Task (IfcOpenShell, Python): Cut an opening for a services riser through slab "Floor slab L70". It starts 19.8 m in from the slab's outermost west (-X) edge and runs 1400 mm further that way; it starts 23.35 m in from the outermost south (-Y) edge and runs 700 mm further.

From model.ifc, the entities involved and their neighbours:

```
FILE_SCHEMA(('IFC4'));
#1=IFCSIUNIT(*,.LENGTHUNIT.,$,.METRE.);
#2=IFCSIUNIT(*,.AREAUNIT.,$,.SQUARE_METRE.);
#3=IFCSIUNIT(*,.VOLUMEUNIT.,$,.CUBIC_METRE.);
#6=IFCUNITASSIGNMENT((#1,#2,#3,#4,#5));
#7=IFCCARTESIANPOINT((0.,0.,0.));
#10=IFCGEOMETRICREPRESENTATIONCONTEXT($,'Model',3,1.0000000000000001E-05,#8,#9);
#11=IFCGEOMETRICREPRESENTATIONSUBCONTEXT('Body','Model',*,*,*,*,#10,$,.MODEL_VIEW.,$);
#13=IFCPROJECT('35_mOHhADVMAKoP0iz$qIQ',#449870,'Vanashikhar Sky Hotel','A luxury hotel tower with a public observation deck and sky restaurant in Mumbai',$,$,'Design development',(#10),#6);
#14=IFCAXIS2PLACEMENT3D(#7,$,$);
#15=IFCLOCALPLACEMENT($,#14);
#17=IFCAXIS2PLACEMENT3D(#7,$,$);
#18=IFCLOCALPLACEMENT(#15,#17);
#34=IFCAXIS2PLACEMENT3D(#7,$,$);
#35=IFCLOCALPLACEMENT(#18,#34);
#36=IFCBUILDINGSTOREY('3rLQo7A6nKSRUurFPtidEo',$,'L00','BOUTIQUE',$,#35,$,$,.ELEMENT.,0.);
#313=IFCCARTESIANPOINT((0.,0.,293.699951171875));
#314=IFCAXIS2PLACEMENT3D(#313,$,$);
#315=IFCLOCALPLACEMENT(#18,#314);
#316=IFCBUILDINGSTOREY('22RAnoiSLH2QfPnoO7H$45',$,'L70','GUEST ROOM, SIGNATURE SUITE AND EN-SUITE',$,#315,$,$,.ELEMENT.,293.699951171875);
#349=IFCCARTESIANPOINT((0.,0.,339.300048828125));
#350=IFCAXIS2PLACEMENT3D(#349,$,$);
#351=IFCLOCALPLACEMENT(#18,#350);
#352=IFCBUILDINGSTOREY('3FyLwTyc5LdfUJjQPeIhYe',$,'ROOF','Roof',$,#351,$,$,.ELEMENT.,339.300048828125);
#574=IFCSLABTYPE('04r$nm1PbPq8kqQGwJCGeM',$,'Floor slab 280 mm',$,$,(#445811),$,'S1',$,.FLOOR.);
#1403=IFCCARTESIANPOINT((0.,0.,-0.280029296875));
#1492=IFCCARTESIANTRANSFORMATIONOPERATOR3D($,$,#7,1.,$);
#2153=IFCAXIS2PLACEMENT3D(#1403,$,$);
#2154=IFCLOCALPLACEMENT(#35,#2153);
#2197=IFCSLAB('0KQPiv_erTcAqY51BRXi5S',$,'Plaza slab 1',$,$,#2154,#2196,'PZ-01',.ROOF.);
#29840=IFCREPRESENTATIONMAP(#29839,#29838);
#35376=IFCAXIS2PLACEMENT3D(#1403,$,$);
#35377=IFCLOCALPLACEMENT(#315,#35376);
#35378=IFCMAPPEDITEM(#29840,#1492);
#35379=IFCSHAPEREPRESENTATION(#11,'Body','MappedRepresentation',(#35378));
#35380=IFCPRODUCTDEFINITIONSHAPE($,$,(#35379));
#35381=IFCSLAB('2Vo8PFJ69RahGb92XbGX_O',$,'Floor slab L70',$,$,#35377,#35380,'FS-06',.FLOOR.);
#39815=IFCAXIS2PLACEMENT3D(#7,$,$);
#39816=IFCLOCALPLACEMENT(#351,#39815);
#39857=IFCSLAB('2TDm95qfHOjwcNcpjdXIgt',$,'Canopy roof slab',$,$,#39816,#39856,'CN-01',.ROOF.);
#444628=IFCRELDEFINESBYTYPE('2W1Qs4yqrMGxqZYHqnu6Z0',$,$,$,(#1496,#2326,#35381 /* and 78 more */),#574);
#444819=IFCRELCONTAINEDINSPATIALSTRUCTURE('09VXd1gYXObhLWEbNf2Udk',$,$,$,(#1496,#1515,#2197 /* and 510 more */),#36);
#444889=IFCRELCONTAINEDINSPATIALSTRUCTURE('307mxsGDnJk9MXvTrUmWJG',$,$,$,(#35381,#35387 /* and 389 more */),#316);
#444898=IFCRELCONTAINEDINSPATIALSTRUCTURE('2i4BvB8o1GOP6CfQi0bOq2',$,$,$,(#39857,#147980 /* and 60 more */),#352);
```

```python
import numpy as np
import ifcopenshell
import ifcopenshell.api.feature
import ifcopenshell.api.geometry
import ifcopenshell.api.root
import ifcopenshell.geom
import ifcopenshell.util.placement
import ifcopenshell.util.representation
import ifcopenshell.util.shape
import ifcopenshell.util.unit

model = ifcopenshell.open("model.ifc")
unit_scale = ifcopenshell.util.unit.calculate_unit_scale(model)
settings = ifcopenshell.geom.settings()


def volume(element):
    """Net volume in cubic metres, openings subtracted."""
    shape = ifcopenshell.geom.create_shape(settings, element)
    return ifcopenshell.util.shape.get_volume(shape.geometry)


slab = model.by_id(35381)
before = volume(slab)

# Extent in the slab's own axes, in metres. The edges named are its -X and -Y sides.
slab_shape = ifcopenshell.geom.create_shape(settings, slab)
vertices = ifcopenshell.util.shape.get_vertices(slab_shape.geometry)
x_min, y_min, bottom = vertices.min(axis=0)
top = vertices[:, 2].max()

opening = ifcopenshell.api.root.create_entity(model, ifc_class="IfcOpeningElement", name="Services riser opening", predefined_type="OPENING")
context = ifcopenshell.util.representation.get_context(model, "Model", "Body", "MODEL_VIEW")
width, depth = 1.4, 0.7
outline = [(0.0, 0.0), (width, 0.0), (width, depth), (0.0, depth), (0.0, 0.0)]
# Overshoot both faces by 50 mm so the cut is clean.
shape = ifcopenshell.api.geometry.add_slab_representation(
    model, context=context, depth=top - bottom + 0.1, polyline=outline
)
ifcopenshell.api.geometry.assign_representation(model, product=opening, representation=shape)

matrix = ifcopenshell.util.placement.get_local_placement(slab.ObjectPlacement)
matrix[:, 3] = matrix @ np.append(np.array([x_min + 19.8, y_min + 23.35, bottom - 0.05]) / unit_scale, 1.0)
ifcopenshell.api.geometry.edit_object_placement(model, product=opening, matrix=matrix, is_si=False)
ifcopenshell.api.feature.add_feature(model, feature=opening, element=slab)

after = volume(slab)

print(f"slab volume {before:.3f} -> {after:.3f} m3")

model.write("model-out.ifc")
```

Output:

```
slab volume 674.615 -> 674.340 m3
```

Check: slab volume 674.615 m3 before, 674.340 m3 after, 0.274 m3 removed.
